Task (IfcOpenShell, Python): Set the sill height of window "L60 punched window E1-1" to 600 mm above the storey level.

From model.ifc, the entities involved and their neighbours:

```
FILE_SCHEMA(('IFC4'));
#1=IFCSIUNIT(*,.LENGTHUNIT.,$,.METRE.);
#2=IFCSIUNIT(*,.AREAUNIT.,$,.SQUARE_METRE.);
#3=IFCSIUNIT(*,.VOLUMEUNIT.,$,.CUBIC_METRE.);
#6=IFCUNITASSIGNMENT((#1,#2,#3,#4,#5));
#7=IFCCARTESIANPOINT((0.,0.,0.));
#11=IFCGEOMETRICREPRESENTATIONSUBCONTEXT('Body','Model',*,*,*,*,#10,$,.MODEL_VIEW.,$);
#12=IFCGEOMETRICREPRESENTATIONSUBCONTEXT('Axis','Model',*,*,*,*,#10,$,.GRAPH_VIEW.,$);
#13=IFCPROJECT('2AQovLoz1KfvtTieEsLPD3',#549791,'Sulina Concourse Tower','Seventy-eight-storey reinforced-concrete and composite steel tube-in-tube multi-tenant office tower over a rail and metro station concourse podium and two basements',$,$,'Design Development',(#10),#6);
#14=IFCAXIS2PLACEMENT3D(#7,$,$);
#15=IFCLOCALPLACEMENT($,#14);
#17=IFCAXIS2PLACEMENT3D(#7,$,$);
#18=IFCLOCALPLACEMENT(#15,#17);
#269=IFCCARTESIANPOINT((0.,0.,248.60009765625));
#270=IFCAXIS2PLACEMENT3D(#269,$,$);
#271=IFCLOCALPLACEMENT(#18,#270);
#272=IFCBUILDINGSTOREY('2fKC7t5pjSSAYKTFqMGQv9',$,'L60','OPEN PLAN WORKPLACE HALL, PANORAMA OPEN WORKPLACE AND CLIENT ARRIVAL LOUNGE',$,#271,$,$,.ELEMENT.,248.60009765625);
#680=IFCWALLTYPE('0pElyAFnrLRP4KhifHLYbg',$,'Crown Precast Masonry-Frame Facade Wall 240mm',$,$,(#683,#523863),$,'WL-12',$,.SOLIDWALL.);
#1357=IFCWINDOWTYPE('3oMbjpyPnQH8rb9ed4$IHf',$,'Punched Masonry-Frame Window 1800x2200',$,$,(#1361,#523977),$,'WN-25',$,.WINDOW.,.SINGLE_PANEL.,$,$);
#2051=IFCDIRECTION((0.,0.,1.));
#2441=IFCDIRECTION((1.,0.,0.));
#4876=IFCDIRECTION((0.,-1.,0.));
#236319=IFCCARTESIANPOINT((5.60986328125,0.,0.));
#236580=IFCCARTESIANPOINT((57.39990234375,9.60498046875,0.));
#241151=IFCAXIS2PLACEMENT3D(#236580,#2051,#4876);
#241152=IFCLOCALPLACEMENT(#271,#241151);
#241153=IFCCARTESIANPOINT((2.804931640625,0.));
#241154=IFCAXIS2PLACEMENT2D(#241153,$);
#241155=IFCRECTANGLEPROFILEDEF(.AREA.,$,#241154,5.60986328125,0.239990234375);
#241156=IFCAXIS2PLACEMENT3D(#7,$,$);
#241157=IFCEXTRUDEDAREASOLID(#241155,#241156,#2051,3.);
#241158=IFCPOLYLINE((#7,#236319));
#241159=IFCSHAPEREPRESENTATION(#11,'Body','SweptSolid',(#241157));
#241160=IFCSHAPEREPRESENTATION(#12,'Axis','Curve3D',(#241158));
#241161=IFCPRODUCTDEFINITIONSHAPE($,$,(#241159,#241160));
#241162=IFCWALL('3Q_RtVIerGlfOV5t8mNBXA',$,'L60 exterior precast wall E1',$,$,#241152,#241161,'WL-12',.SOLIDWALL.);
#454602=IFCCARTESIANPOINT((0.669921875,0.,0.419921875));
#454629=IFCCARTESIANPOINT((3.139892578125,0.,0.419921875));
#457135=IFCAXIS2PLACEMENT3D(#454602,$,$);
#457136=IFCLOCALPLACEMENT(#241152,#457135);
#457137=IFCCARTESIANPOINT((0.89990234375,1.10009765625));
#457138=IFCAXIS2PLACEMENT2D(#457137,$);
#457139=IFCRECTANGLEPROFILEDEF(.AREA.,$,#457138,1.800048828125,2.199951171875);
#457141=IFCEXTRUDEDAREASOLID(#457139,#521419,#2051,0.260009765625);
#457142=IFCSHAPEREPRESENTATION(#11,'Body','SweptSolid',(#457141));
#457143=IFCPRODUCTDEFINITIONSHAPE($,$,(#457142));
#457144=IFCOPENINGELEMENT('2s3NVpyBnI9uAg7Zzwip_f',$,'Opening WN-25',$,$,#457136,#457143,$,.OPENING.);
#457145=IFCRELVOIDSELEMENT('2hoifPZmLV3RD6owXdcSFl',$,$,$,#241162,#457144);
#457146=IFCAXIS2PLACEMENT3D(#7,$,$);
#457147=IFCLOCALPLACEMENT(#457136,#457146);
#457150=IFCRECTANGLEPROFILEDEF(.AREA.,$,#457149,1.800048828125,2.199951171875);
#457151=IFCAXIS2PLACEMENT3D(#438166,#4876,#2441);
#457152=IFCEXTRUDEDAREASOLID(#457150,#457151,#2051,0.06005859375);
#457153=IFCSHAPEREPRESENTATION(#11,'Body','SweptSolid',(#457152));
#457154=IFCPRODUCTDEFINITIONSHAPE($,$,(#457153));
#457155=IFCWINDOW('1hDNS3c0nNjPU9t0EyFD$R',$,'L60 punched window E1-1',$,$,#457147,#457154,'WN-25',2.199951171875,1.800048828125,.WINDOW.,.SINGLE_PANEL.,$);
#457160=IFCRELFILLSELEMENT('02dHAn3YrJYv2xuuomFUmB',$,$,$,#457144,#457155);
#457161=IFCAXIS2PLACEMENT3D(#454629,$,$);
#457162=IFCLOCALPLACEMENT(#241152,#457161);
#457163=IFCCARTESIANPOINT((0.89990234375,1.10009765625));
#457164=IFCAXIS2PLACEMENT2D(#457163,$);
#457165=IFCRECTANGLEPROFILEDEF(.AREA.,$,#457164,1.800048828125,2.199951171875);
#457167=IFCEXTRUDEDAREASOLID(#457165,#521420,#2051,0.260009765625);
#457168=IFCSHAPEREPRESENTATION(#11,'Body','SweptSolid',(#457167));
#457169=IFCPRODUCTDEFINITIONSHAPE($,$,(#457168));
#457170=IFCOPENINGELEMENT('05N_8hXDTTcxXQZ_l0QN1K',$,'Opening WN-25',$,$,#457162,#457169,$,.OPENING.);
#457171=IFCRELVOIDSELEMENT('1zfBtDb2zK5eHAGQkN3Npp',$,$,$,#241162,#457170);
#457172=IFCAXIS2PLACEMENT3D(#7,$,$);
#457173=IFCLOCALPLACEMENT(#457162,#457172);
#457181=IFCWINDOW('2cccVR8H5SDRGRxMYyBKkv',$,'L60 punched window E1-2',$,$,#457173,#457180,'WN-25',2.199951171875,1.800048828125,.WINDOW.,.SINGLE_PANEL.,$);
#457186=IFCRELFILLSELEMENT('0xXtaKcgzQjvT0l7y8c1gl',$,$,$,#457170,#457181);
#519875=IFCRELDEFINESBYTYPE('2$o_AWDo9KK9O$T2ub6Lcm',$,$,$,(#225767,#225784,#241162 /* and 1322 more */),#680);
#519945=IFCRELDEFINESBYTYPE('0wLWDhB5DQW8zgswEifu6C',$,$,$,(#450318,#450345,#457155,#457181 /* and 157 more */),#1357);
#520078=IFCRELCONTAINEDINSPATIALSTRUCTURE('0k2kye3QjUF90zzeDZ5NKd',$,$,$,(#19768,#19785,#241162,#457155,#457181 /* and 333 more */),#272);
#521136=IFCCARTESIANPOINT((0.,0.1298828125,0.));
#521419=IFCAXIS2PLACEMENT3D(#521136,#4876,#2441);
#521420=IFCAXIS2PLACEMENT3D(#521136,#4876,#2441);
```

```python
import numpy as np
import ifcopenshell
import ifcopenshell.api.geometry
import ifcopenshell.geom
import ifcopenshell.util.element
import ifcopenshell.util.placement
import ifcopenshell.util.shape
import ifcopenshell.util.unit

model = ifcopenshell.open("model.ifc")
unit_scale = ifcopenshell.util.unit.calculate_unit_scale(model)

window = model.by_guid("1hDNS3c0nNjPU9t0EyFD$R")
opening = window.FillsVoids[0].RelatingOpeningElement
storey = ifcopenshell.util.element.get_container(window, ifc_class="IfcBuildingStorey")
level = ifcopenshell.util.placement.get_local_placement(storey.ObjectPlacement)[2, 3]

# The opening's origin need not be at the sill, so measure its lowest point.
shape = ifcopenshell.geom.create_shape(ifcopenshell.geom.settings(), opening)
bottom = ifcopenshell.util.shape.get_shape_bottom_elevation(shape, shape.geometry) / unit_scale
dz = level + 0.6 - bottom

shift = np.array([0.0, 0.0, dz])
# The window is placed relative to its opening, so it follows when the opening moves.
matrix = ifcopenshell.util.placement.get_local_placement(opening.ObjectPlacement)
matrix[:3, 3] += shift
ifcopenshell.api.geometry.edit_object_placement(
    model, product=opening, matrix=matrix, is_si=False, should_transform_children=True
)

print(f"moved by {dz * unit_scale:+.3f} m")

model.write("model_v2.ifc")
```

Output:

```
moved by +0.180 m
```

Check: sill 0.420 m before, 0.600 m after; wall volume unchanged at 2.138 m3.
